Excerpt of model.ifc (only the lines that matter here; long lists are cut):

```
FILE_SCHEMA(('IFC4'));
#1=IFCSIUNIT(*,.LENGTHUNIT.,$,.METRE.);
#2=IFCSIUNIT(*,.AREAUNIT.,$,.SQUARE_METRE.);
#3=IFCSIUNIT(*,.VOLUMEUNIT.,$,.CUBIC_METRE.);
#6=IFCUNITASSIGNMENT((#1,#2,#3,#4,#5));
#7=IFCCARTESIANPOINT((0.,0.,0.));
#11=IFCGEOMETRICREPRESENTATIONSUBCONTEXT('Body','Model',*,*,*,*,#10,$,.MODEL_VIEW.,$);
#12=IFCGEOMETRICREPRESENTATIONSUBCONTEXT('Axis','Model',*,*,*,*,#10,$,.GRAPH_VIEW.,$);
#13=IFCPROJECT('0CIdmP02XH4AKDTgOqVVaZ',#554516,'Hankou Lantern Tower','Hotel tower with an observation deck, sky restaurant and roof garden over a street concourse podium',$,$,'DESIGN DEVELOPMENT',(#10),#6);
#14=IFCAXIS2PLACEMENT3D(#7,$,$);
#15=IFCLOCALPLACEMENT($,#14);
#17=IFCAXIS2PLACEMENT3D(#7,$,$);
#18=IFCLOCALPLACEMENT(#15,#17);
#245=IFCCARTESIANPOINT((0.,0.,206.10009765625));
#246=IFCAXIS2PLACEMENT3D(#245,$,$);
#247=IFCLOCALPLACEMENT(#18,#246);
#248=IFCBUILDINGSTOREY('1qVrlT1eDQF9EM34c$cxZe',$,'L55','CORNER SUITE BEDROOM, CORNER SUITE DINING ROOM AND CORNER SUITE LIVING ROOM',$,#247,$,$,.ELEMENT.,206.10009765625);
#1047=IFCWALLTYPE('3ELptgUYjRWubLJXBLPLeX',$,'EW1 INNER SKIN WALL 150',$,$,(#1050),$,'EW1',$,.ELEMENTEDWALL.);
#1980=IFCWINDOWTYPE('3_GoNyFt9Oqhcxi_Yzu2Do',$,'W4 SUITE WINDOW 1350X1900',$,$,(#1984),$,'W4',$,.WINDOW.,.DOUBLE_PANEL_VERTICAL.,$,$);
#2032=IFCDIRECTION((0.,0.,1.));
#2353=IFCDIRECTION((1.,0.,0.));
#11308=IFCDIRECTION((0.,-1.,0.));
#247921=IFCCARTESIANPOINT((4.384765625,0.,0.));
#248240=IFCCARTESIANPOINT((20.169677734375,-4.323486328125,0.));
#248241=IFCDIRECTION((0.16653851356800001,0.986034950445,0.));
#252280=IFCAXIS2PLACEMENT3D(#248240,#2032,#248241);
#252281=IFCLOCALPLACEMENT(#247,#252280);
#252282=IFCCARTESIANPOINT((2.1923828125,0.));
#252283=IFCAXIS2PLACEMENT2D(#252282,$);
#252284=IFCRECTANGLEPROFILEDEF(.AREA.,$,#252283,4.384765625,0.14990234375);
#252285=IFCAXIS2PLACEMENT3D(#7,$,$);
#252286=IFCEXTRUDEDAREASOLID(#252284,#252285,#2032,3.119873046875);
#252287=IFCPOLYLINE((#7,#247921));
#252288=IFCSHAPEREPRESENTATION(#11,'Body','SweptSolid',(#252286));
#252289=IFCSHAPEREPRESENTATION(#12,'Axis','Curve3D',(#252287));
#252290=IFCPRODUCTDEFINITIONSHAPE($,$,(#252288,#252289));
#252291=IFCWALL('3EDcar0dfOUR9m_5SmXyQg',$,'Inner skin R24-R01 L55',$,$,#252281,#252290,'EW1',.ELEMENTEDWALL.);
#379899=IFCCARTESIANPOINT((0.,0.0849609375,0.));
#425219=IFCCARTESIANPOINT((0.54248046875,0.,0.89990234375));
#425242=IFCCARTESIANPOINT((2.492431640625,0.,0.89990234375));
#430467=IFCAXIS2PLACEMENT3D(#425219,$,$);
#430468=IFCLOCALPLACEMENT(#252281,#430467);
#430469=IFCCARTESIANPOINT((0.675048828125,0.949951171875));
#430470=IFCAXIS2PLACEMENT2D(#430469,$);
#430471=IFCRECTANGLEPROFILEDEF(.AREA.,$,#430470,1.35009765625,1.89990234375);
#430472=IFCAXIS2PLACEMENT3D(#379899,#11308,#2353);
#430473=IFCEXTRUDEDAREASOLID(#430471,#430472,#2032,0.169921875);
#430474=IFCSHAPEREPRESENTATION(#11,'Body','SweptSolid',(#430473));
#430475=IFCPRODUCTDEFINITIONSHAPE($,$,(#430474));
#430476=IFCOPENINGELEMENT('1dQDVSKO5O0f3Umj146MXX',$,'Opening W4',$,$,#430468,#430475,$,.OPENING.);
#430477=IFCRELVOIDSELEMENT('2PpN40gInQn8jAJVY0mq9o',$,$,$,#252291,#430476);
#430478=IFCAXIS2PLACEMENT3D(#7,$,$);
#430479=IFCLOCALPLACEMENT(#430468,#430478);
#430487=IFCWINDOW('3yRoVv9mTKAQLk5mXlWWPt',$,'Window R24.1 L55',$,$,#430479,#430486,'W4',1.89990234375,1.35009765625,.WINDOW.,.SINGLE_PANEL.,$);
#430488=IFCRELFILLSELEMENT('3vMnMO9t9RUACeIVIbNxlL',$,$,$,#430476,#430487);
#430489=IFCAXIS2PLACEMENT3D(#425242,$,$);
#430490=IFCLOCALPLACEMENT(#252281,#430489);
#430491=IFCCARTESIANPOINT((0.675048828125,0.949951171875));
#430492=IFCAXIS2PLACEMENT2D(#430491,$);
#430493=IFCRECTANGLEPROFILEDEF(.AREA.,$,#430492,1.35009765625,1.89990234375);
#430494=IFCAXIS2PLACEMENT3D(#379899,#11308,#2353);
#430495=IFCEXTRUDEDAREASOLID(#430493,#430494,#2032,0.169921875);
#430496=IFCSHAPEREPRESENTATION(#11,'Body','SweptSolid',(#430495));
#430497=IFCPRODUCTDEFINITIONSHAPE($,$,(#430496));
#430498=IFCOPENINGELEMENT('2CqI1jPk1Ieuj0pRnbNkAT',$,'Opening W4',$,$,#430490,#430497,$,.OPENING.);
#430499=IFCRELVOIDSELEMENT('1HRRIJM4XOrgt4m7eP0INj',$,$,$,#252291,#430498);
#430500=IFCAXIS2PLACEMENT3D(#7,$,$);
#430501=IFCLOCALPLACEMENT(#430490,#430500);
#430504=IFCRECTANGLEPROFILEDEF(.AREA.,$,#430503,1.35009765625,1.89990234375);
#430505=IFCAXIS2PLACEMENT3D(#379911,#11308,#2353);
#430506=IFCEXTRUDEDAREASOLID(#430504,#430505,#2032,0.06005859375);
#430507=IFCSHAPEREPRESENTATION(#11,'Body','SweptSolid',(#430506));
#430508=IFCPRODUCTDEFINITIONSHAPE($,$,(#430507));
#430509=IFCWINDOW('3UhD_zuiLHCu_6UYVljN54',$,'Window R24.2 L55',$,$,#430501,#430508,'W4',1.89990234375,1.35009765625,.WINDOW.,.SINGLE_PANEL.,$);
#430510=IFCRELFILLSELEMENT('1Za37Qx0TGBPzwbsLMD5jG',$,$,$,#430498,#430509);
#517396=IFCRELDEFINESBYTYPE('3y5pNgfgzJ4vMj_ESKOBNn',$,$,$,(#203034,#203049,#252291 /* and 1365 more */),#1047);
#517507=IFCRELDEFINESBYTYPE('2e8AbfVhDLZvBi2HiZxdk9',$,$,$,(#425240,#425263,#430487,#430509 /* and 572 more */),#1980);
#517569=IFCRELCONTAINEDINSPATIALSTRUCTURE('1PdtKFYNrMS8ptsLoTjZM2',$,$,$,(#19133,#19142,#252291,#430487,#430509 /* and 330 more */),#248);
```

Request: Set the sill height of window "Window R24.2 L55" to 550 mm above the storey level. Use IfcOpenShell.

```python
import numpy as np
import ifcopenshell
import ifcopenshell.api.geometry
import ifcopenshell.geom
import ifcopenshell.util.element
import ifcopenshell.util.placement
import ifcopenshell.util.shape
import ifcopenshell.util.unit

model = ifcopenshell.open("model.ifc")
unit_scale = ifcopenshell.util.unit.calculate_unit_scale(model)

window = model.by_id(430509)
opening = window.FillsVoids[0].RelatingOpeningElement
storey = ifcopenshell.util.element.get_container(window, ifc_class="IfcBuildingStorey")
level = ifcopenshell.util.placement.get_local_placement(storey.ObjectPlacement)[2, 3]

# The opening's origin need not be at the sill, so measure its lowest point.
shape = ifcopenshell.geom.create_shape(ifcopenshell.geom.settings(), opening)
bottom = ifcopenshell.util.shape.get_shape_bottom_elevation(shape, shape.geometry) / unit_scale
dz = level + 0.55 - bottom

shift = np.array([0.0, 0.0, dz])
# The window is placed relative to its opening, so it follows when the opening moves.
matrix = ifcopenshell.util.placement.get_local_placement(opening.ObjectPlacement)
matrix[:3, 3] += shift
ifcopenshell.api.geometry.edit_object_placement(
    model, product=opening, matrix=matrix, is_si=False, should_transform_children=True
)

print(f"moved by {dz * unit_scale:+.3f} m")

model.write("model_rev.ifc")
```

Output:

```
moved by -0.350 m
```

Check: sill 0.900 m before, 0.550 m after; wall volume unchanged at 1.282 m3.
